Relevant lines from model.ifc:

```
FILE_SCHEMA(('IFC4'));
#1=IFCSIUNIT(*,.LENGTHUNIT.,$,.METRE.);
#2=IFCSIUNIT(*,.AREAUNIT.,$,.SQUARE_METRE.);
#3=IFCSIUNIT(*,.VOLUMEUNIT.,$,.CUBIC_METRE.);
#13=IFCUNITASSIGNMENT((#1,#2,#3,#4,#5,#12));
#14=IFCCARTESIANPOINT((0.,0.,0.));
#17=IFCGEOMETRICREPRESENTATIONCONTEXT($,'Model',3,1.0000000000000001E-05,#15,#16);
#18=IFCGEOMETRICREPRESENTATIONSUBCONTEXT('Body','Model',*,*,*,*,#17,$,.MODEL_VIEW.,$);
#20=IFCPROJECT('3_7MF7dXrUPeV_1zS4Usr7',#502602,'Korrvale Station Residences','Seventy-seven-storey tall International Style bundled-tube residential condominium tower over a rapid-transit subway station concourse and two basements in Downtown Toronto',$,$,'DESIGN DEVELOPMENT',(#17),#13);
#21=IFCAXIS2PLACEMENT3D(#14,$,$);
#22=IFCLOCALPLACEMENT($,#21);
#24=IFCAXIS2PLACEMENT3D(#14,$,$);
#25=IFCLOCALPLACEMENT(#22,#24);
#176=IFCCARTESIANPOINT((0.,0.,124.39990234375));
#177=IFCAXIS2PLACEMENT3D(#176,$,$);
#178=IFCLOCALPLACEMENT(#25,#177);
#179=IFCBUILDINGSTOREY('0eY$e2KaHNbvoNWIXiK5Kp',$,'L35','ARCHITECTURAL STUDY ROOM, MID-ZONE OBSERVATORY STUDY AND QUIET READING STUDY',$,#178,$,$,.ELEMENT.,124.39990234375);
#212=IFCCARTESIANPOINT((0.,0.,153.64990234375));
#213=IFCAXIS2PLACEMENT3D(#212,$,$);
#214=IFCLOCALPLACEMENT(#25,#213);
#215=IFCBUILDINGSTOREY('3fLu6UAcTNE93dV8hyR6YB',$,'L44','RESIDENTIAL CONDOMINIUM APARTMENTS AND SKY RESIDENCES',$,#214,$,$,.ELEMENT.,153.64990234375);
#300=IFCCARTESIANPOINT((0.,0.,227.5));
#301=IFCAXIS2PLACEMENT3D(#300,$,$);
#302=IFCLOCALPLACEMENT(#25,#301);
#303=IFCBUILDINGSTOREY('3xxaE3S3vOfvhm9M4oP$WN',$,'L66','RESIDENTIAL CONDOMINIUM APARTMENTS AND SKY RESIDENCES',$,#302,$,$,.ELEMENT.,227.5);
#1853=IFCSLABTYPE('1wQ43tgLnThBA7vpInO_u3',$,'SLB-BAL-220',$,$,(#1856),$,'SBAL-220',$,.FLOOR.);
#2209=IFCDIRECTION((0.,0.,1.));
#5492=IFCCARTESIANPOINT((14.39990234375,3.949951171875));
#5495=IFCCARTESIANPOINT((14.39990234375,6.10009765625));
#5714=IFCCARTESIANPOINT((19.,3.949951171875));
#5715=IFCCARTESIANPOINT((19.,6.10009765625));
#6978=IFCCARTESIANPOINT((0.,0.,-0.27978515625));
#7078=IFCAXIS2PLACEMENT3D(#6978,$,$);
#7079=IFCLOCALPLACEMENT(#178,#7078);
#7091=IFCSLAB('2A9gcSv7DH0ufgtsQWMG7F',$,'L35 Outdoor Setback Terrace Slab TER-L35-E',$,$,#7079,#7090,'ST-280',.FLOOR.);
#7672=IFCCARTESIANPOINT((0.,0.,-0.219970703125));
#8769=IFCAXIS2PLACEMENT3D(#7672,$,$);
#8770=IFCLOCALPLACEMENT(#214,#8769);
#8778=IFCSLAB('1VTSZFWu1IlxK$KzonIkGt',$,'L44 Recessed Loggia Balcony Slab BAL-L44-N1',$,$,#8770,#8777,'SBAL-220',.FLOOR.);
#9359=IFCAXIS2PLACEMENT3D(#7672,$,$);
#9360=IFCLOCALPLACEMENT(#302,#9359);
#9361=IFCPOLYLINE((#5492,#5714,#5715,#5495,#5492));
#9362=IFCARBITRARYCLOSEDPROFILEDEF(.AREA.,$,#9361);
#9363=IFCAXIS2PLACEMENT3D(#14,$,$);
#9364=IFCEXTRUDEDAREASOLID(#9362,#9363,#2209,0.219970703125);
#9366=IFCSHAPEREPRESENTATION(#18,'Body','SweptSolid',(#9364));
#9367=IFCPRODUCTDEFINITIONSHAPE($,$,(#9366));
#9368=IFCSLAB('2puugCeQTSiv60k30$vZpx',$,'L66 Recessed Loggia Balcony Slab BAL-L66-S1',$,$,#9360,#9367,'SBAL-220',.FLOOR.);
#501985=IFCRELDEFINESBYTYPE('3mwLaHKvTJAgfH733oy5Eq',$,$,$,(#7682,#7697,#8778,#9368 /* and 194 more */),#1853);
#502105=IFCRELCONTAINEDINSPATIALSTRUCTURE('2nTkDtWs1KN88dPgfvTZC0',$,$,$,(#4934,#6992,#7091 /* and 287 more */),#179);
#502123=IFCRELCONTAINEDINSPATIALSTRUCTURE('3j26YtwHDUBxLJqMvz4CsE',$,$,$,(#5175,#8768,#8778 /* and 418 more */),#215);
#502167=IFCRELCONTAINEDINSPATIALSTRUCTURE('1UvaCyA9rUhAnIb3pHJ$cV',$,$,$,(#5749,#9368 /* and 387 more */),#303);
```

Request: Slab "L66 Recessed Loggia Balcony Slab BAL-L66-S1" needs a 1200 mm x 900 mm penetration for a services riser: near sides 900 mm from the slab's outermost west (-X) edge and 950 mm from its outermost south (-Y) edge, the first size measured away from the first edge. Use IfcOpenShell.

```python
import numpy as np
import ifcopenshell
import ifcopenshell.api.feature
import ifcopenshell.api.geometry
import ifcopenshell.api.root
import ifcopenshell.geom
import ifcopenshell.util.placement
import ifcopenshell.util.representation
import ifcopenshell.util.shape
import ifcopenshell.util.unit

model = ifcopenshell.open("model.ifc")
unit_scale = ifcopenshell.util.unit.calculate_unit_scale(model)
settings = ifcopenshell.geom.settings()


def volume(element):
    """Net volume in cubic metres, openings subtracted."""
    shape = ifcopenshell.geom.create_shape(settings, element)
    return ifcopenshell.util.shape.get_volume(shape.geometry)


slab = model.by_id(9368)
before = volume(slab)

# Extent in the slab's own axes, in metres. The edges named are its -X and -Y sides.
slab_shape = ifcopenshell.geom.create_shape(settings, slab)
vertices = ifcopenshell.util.shape.get_vertices(slab_shape.geometry)
x_min, y_min, bottom = vertices.min(axis=0)
top = vertices[:, 2].max()

opening = ifcopenshell.api.root.create_entity(model, ifc_class="IfcOpeningElement", name="Services riser opening", predefined_type="OPENING")
context = ifcopenshell.util.representation.get_context(model, "Model", "Body", "MODEL_VIEW")
width, depth = 1.2, 0.9
outline = [(0.0, 0.0), (width, 0.0), (width, depth), (0.0, depth), (0.0, 0.0)]
# Overshoot both faces by 50 mm so the cut is clean.
shape = ifcopenshell.api.geometry.add_slab_representation(
    model, context=context, depth=top - bottom + 0.1, polyline=outline
)
ifcopenshell.api.geometry.assign_representation(model, product=opening, representation=shape)

matrix = ifcopenshell.util.placement.get_local_placement(slab.ObjectPlacement)
matrix[:, 3] = matrix @ np.append(np.array([x_min + 0.9, y_min + 0.95, bottom - 0.05]) / unit_scale, 1.0)
ifcopenshell.api.geometry.edit_object_placement(model, product=opening, matrix=matrix, is_si=False)
ifcopenshell.api.feature.add_feature(model, feature=opening, element=slab)

after = volume(slab)

print(f"slab volume {before:.3f} -> {after:.3f} m3")

model.write("model_edited.ifc")
```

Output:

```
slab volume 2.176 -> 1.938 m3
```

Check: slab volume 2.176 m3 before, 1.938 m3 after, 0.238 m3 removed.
